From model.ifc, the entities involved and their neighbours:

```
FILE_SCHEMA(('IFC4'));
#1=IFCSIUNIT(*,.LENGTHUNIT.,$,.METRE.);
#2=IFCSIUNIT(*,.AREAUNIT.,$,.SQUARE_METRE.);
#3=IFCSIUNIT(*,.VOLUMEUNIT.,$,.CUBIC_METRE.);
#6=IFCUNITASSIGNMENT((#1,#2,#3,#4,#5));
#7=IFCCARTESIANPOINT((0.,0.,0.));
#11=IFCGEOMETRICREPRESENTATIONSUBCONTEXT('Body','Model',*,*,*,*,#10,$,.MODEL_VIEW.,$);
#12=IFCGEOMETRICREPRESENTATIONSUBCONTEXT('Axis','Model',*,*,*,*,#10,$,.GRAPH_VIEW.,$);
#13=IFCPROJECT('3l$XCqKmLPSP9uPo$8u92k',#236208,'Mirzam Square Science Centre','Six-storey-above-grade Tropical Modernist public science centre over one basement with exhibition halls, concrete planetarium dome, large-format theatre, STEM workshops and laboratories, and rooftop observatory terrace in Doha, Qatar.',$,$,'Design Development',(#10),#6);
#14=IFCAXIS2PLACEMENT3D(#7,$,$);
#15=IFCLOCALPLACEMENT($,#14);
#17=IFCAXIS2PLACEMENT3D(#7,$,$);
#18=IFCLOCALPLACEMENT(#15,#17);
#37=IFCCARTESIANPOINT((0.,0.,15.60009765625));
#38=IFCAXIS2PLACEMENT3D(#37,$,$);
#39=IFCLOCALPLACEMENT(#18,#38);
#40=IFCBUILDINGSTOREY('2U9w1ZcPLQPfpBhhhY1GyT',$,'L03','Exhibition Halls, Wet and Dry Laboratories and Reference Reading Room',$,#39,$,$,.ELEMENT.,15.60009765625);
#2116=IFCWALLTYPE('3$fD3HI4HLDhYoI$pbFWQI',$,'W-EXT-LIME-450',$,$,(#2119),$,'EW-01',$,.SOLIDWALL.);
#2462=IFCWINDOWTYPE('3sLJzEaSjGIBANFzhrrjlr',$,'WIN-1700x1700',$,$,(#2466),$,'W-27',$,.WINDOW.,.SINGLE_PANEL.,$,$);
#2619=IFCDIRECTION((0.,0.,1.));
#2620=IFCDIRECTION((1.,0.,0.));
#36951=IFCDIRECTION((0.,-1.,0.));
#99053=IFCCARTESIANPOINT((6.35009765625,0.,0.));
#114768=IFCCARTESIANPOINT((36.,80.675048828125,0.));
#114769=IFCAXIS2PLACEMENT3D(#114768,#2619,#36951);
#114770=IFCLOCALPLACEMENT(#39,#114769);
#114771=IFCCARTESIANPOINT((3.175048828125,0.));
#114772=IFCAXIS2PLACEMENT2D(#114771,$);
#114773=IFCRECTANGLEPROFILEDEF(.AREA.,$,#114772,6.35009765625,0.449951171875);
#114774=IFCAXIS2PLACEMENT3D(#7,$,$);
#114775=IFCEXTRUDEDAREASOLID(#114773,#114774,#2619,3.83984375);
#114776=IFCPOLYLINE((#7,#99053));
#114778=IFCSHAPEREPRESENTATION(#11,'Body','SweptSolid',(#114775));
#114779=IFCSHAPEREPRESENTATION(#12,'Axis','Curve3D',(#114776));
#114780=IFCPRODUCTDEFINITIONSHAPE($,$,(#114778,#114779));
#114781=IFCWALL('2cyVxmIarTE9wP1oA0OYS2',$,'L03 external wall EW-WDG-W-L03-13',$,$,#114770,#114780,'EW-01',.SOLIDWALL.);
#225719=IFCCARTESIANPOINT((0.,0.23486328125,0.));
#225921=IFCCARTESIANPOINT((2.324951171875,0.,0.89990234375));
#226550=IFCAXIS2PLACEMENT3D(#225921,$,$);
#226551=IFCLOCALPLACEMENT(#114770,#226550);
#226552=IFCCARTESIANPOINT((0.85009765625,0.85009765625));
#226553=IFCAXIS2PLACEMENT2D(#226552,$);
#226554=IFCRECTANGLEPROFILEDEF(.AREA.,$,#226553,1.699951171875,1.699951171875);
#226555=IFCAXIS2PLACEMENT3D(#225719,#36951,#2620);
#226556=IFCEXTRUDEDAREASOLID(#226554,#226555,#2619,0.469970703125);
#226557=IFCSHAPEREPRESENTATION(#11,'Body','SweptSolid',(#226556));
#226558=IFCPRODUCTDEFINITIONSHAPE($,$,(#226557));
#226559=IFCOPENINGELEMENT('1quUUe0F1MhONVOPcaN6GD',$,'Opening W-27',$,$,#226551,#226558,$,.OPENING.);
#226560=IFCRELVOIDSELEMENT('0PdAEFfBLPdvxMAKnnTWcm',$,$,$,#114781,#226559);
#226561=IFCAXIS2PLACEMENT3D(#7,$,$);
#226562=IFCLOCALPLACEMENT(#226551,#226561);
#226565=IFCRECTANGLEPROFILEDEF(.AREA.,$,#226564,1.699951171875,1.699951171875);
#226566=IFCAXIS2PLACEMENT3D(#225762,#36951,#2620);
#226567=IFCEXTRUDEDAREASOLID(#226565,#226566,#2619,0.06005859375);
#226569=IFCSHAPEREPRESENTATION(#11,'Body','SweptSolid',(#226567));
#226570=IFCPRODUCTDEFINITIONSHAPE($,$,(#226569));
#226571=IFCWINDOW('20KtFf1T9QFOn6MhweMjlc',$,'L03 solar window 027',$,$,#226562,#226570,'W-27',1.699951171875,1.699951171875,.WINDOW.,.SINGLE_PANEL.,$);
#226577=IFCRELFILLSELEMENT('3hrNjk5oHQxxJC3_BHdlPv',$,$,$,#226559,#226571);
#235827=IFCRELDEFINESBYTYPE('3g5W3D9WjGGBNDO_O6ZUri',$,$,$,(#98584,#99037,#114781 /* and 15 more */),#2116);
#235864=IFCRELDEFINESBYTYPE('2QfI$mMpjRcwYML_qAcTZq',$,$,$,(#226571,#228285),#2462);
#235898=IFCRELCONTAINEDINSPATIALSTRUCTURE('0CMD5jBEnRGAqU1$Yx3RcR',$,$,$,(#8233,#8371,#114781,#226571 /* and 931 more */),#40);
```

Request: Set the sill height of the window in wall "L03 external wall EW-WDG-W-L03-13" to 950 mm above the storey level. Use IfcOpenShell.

```python
import numpy as np
import ifcopenshell
import ifcopenshell.api.geometry
import ifcopenshell.geom
import ifcopenshell.util.element
import ifcopenshell.util.placement
import ifcopenshell.util.shape
import ifcopenshell.util.unit

model = ifcopenshell.open("model.ifc")
unit_scale = ifcopenshell.util.unit.calculate_unit_scale(model)

window = model.by_guid("20KtFf1T9QFOn6MhweMjlc")
opening = window.FillsVoids[0].RelatingOpeningElement
storey = ifcopenshell.util.element.get_container(window, ifc_class="IfcBuildingStorey")
level = ifcopenshell.util.placement.get_local_placement(storey.ObjectPlacement)[2, 3]

# The opening's origin need not be at the sill, so measure its lowest point.
shape = ifcopenshell.geom.create_shape(ifcopenshell.geom.settings(), opening)
bottom = ifcopenshell.util.shape.get_shape_bottom_elevation(shape, shape.geometry) / unit_scale
dz = level + 0.95 / unit_scale - bottom

shift = np.array([0.0, 0.0, dz])
# The window is placed relative to its opening, so it follows when the opening moves.
matrix = ifcopenshell.util.placement.get_local_placement(opening.ObjectPlacement)
matrix[:3, 3] += shift
ifcopenshell.api.geometry.edit_object_placement(
    model, product=opening, matrix=matrix, is_si=False, should_transform_children=True
)

print(f"moved by {dz * unit_scale:+.3f} m")

model.write("model_edited.ifc")
```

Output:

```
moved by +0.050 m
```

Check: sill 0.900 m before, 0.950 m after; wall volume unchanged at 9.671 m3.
